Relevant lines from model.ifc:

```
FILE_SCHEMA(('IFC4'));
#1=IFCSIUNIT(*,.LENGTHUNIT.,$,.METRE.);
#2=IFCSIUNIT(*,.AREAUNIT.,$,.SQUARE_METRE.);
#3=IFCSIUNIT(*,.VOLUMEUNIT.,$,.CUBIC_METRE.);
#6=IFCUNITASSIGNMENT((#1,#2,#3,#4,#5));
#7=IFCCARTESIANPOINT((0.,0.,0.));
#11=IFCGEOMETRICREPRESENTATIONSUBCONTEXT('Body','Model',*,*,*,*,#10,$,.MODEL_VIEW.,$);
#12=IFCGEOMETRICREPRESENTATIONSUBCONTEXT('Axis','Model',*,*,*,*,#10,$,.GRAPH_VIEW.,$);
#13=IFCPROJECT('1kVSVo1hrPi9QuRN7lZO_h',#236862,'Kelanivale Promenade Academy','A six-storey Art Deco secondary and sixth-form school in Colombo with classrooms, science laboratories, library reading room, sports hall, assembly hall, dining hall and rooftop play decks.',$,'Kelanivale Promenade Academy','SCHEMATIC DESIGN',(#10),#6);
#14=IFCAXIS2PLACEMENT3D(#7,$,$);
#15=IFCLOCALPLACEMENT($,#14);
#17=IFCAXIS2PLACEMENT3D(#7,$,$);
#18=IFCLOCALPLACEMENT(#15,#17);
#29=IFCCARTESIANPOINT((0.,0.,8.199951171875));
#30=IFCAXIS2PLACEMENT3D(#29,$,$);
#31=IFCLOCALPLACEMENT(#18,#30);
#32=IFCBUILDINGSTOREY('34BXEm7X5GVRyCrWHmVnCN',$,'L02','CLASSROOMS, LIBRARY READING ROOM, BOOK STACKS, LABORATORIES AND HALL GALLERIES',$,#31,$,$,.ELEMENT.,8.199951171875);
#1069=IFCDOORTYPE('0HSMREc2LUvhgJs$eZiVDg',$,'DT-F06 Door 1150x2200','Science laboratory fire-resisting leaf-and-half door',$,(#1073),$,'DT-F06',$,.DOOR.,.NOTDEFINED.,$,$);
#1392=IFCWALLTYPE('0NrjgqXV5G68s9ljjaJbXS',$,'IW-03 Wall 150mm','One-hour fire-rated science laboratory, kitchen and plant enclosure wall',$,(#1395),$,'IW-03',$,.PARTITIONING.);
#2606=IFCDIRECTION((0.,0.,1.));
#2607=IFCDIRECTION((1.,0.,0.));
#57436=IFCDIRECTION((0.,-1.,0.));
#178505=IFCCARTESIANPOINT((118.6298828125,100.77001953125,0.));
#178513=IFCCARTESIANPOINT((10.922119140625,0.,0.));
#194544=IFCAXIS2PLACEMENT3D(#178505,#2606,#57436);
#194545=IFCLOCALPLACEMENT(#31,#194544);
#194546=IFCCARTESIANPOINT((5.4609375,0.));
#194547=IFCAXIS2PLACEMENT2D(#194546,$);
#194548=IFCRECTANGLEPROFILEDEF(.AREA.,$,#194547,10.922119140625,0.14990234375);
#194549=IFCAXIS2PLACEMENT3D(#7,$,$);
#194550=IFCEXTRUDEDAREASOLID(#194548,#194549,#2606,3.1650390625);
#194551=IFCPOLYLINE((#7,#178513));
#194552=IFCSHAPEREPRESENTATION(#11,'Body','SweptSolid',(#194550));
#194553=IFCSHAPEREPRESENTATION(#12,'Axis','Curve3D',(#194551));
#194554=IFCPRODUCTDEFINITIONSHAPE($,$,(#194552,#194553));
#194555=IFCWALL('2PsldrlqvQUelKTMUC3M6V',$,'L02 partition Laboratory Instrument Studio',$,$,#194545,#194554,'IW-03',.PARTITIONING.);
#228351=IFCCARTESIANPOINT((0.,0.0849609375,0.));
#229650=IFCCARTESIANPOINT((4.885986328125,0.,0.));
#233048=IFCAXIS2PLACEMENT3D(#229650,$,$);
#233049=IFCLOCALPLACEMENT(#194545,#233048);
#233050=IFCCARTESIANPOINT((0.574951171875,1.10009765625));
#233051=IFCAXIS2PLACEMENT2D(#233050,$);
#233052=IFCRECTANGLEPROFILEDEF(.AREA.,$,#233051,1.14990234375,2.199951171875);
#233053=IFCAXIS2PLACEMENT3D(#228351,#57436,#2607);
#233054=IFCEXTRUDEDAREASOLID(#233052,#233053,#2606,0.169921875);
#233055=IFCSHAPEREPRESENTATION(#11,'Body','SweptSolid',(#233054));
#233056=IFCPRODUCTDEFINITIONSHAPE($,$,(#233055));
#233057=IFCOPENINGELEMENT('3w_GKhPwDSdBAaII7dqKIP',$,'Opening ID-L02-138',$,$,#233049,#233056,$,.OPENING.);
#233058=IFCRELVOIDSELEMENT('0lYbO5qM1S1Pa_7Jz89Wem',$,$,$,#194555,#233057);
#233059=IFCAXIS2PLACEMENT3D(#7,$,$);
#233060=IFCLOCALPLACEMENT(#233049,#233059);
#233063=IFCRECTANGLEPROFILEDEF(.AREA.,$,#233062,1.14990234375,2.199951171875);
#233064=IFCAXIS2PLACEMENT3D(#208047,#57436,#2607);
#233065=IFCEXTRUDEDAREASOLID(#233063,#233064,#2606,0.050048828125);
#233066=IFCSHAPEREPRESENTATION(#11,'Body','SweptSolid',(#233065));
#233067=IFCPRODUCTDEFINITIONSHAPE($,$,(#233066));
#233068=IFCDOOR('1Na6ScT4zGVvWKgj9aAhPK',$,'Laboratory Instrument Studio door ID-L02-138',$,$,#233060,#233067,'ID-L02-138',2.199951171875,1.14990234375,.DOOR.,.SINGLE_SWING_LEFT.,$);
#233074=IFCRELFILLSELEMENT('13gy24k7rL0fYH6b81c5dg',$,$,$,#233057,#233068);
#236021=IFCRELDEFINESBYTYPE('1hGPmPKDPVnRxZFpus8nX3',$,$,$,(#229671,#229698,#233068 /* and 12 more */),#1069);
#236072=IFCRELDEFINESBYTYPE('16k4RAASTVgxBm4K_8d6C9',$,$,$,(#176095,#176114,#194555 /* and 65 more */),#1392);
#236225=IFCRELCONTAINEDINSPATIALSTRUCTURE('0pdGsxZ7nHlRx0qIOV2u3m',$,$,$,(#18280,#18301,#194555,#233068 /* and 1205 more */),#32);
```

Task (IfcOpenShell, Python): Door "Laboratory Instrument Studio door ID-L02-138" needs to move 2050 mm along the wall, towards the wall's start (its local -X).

```python
import ifcopenshell
import ifcopenshell.api.geometry
import ifcopenshell.util.placement
import ifcopenshell.util.unit

model = ifcopenshell.open("model.ifc")
unit_scale = ifcopenshell.util.unit.calculate_unit_scale(model)

door = model.by_guid("1Na6ScT4zGVvWKgj9aAhPK")
opening = door.FillsVoids[0].RelatingOpeningElement
wall = opening.VoidsElements[0].RelatingBuildingElement

wall_matrix = ifcopenshell.util.placement.get_local_placement(wall.ObjectPlacement)
shift = wall_matrix[:3, 0] * -2.05 / unit_scale
before = ifcopenshell.util.placement.get_local_placement(door.ObjectPlacement)[:3, 3].copy()

# The door is placed relative to its opening, so it follows when the opening moves.
matrix = ifcopenshell.util.placement.get_local_placement(opening.ObjectPlacement)
matrix[:3, 3] += shift
ifcopenshell.api.geometry.edit_object_placement(
    model, product=opening, matrix=matrix, is_si=False, should_transform_children=True
)

after = ifcopenshell.util.placement.get_local_placement(door.ObjectPlacement)[:3, 3]
print("door moved by", (after - before).round(3) + 0.0)

model.write("model-out.ifc")
```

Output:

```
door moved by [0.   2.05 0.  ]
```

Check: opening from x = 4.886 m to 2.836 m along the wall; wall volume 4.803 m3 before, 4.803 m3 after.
